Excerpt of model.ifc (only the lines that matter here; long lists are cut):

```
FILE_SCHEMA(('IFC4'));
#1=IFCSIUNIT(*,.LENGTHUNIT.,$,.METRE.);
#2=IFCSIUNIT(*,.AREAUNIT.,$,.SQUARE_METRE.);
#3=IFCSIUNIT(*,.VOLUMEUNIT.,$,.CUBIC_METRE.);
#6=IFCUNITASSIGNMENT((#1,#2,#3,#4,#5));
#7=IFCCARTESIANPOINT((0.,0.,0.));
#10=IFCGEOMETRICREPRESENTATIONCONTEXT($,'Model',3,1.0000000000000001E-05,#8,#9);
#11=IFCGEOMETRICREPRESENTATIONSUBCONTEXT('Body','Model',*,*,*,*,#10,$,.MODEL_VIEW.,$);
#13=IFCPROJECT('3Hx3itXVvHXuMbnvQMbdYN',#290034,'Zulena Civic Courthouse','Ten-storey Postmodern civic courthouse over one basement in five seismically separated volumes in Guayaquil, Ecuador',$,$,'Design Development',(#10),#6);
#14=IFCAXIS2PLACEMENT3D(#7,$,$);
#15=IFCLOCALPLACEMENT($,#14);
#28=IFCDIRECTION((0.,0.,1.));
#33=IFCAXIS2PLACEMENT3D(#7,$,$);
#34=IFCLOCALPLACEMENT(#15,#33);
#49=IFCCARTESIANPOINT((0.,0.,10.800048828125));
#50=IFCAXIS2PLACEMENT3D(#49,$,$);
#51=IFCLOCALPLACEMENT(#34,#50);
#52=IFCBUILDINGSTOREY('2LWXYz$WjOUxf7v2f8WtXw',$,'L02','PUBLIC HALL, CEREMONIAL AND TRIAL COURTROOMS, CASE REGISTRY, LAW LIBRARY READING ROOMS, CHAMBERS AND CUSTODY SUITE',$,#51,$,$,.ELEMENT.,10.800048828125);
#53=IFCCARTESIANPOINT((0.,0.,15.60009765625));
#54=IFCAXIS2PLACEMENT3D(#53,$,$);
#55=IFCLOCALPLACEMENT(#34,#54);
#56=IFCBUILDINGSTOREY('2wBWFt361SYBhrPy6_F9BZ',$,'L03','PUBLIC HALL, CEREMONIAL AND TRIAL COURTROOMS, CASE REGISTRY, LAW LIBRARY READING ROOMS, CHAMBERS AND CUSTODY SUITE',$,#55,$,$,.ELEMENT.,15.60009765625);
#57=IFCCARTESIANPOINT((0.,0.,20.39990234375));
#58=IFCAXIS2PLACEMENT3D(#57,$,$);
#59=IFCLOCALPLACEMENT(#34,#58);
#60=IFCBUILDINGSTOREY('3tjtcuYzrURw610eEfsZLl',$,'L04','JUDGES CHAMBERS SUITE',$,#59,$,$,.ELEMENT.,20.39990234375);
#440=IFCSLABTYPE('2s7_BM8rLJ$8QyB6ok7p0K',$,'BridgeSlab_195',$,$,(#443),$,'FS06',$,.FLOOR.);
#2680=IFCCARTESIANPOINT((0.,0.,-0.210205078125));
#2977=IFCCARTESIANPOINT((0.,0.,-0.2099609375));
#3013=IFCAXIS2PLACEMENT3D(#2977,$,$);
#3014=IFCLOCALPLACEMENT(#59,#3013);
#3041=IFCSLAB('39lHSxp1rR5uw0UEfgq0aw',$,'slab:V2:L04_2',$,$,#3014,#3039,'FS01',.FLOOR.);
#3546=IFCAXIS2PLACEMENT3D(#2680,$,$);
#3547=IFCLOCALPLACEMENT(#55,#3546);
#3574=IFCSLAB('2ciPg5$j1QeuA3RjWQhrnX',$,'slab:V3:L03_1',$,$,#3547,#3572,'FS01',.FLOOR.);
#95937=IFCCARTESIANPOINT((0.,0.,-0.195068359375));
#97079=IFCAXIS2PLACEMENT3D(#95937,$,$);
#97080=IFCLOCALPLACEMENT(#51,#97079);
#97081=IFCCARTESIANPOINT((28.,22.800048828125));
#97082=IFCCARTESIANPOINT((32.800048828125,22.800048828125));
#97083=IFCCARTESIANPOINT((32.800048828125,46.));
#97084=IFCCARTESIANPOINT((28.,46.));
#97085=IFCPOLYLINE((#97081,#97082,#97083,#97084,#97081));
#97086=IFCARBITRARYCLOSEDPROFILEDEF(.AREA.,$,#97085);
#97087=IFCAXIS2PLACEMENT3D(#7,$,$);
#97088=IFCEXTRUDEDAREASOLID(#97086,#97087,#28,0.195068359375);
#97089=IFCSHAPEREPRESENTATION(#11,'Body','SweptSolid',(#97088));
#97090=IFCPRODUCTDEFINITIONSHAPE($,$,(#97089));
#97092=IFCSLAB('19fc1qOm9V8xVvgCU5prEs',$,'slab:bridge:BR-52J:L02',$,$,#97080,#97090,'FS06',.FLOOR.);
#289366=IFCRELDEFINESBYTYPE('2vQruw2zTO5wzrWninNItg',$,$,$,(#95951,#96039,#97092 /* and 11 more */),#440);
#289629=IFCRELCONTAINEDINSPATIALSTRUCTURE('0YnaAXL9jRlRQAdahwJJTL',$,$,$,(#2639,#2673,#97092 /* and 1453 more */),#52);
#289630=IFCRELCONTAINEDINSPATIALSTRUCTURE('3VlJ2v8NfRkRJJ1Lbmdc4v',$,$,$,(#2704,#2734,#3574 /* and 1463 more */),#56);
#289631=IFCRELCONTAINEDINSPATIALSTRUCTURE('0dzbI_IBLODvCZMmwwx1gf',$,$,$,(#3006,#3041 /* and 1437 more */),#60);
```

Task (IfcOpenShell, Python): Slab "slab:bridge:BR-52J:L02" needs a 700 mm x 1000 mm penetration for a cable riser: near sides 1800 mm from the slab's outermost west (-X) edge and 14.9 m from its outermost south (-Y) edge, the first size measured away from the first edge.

```python
import numpy as np
import ifcopenshell
import ifcopenshell.api.feature
import ifcopenshell.api.geometry
import ifcopenshell.api.root
import ifcopenshell.geom
import ifcopenshell.util.placement
import ifcopenshell.util.representation
import ifcopenshell.util.shape
import ifcopenshell.util.unit

model = ifcopenshell.open("model.ifc")
unit_scale = ifcopenshell.util.unit.calculate_unit_scale(model)
settings = ifcopenshell.geom.settings()


def volume(element):
    """Net volume in cubic metres, openings subtracted."""
    shape = ifcopenshell.geom.create_shape(settings, element)
    return ifcopenshell.util.shape.get_volume(shape.geometry)


slab = model.by_guid("19fc1qOm9V8xVvgCU5prEs")
before = volume(slab)

# Extent in the slab's own axes, in metres. The edges named are its -X and -Y sides.
slab_shape = ifcopenshell.geom.create_shape(settings, slab)
vertices = ifcopenshell.util.shape.get_vertices(slab_shape.geometry)
x_min, y_min, bottom = vertices.min(axis=0)
top = vertices[:, 2].max()

opening = ifcopenshell.api.root.create_entity(model, ifc_class="IfcOpeningElement", name="Cable riser opening", predefined_type="OPENING")
context = ifcopenshell.util.representation.get_context(model, "Model", "Body", "MODEL_VIEW")
width, depth = 0.7, 1
outline = [(0.0, 0.0), (width, 0.0), (width, depth), (0.0, depth), (0.0, 0.0)]
# Overshoot both faces by 50 mm so the cut is clean.
shape = ifcopenshell.api.geometry.add_slab_representation(
    model, context=context, depth=top - bottom + 0.1, polyline=outline
)
ifcopenshell.api.geometry.assign_representation(model, product=opening, representation=shape)

matrix = ifcopenshell.util.placement.get_local_placement(slab.ObjectPlacement)
matrix[:, 3] = matrix @ np.append(np.array([x_min + 1.8, y_min + 14.9, bottom - 0.05]) / unit_scale, 1.0)
ifcopenshell.api.geometry.edit_object_placement(model, product=opening, matrix=matrix, is_si=False)
ifcopenshell.api.feature.add_feature(model, feature=opening, element=slab)

after = volume(slab)

print(f"slab volume {before:.3f} -> {after:.3f} m3")

model.write("model-out.ifc")
```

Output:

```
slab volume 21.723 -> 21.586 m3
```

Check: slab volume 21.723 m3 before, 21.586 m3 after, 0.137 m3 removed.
